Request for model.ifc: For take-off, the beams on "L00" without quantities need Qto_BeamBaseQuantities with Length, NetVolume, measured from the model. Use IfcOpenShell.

First a look at what the model holds.

```python
import ifcopenshell
import ifcopenshell.util.element
import ifcopenshell.util.unit

model = ifcopenshell.open("model.ifc")
print(model.schema)
for unit_type in ("LENGTHUNIT", "AREAUNIT", "VOLUMEUNIT"):
    print(unit_type, ifcopenshell.util.unit.calculate_unit_scale(model, unit_type))
storey = next(s for s in model.by_type("IfcBuildingStorey") if s.Name == "L00")
beams = [e for e in ifcopenshell.util.element.get_decomposition(storey) if e.is_a("IfcBeam")]
for e in sorted(beams, key=lambda e: e.id()):
    print(e.id(), e.is_a(), e.Name, list(ifcopenshell.util.element.get_psets(e, qtos_only=True)), sep=" | ")
```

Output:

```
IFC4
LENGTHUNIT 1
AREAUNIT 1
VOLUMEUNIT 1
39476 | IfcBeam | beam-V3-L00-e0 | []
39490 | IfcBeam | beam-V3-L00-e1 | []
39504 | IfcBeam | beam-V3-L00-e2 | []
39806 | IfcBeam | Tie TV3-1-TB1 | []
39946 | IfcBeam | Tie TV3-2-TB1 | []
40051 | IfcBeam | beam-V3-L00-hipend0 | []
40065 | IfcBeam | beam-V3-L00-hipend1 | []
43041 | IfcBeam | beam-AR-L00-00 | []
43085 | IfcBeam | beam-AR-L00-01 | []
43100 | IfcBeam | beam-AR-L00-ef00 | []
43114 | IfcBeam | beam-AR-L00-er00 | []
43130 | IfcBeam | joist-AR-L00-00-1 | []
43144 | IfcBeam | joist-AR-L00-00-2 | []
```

```python
import ifcopenshell
import ifcopenshell.api.pset
import ifcopenshell.geom
import ifcopenshell.util.element
import ifcopenshell.util.shape
import ifcopenshell.util.unit

model = ifcopenshell.open("model.ifc")
unit_scale = ifcopenshell.util.unit.calculate_unit_scale(model)
volume_scale = ifcopenshell.util.unit.calculate_unit_scale(model, "VOLUMEUNIT")
settings = ifcopenshell.geom.settings()

storey = next(s for s in model.by_type("IfcBuildingStorey") if s.Name == "L00")
beams = [e for e in ifcopenshell.util.element.get_decomposition(storey) if e.is_a("IfcBeam")]

for e in sorted(beams, key=lambda e: e.id()):
    if ifcopenshell.util.element.get_psets(e, qtos_only=True, should_inherit=False):
        continue
    # Geometry comes back in metres, in the element's own axes.
    shape = ifcopenshell.geom.create_shape(settings, e)
    values = {
        "Length": ifcopenshell.util.shape.get_max_xyz(shape.geometry) / unit_scale,
        "NetVolume": ifcopenshell.util.shape.get_volume(shape.geometry) / volume_scale,
    }
    qto = ifcopenshell.api.pset.add_qto(model, product=e, name="Qto_BeamBaseQuantities")
    ifcopenshell.api.pset.edit_qto(model, qto=qto, properties=values)
    print(e.id(), {k: round(v, 3) for k, v in values.items()})

model.write("model_updated.ifc")
```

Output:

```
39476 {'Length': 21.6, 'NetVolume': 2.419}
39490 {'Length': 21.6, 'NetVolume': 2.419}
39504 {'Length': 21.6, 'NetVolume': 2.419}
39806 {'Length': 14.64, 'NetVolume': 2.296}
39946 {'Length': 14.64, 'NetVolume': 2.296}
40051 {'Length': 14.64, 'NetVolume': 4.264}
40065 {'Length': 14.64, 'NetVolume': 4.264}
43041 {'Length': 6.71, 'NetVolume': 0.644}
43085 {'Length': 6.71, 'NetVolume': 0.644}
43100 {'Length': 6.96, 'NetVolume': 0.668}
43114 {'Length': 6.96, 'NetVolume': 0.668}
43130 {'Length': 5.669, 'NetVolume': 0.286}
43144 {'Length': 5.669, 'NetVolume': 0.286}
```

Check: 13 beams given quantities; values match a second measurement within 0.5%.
